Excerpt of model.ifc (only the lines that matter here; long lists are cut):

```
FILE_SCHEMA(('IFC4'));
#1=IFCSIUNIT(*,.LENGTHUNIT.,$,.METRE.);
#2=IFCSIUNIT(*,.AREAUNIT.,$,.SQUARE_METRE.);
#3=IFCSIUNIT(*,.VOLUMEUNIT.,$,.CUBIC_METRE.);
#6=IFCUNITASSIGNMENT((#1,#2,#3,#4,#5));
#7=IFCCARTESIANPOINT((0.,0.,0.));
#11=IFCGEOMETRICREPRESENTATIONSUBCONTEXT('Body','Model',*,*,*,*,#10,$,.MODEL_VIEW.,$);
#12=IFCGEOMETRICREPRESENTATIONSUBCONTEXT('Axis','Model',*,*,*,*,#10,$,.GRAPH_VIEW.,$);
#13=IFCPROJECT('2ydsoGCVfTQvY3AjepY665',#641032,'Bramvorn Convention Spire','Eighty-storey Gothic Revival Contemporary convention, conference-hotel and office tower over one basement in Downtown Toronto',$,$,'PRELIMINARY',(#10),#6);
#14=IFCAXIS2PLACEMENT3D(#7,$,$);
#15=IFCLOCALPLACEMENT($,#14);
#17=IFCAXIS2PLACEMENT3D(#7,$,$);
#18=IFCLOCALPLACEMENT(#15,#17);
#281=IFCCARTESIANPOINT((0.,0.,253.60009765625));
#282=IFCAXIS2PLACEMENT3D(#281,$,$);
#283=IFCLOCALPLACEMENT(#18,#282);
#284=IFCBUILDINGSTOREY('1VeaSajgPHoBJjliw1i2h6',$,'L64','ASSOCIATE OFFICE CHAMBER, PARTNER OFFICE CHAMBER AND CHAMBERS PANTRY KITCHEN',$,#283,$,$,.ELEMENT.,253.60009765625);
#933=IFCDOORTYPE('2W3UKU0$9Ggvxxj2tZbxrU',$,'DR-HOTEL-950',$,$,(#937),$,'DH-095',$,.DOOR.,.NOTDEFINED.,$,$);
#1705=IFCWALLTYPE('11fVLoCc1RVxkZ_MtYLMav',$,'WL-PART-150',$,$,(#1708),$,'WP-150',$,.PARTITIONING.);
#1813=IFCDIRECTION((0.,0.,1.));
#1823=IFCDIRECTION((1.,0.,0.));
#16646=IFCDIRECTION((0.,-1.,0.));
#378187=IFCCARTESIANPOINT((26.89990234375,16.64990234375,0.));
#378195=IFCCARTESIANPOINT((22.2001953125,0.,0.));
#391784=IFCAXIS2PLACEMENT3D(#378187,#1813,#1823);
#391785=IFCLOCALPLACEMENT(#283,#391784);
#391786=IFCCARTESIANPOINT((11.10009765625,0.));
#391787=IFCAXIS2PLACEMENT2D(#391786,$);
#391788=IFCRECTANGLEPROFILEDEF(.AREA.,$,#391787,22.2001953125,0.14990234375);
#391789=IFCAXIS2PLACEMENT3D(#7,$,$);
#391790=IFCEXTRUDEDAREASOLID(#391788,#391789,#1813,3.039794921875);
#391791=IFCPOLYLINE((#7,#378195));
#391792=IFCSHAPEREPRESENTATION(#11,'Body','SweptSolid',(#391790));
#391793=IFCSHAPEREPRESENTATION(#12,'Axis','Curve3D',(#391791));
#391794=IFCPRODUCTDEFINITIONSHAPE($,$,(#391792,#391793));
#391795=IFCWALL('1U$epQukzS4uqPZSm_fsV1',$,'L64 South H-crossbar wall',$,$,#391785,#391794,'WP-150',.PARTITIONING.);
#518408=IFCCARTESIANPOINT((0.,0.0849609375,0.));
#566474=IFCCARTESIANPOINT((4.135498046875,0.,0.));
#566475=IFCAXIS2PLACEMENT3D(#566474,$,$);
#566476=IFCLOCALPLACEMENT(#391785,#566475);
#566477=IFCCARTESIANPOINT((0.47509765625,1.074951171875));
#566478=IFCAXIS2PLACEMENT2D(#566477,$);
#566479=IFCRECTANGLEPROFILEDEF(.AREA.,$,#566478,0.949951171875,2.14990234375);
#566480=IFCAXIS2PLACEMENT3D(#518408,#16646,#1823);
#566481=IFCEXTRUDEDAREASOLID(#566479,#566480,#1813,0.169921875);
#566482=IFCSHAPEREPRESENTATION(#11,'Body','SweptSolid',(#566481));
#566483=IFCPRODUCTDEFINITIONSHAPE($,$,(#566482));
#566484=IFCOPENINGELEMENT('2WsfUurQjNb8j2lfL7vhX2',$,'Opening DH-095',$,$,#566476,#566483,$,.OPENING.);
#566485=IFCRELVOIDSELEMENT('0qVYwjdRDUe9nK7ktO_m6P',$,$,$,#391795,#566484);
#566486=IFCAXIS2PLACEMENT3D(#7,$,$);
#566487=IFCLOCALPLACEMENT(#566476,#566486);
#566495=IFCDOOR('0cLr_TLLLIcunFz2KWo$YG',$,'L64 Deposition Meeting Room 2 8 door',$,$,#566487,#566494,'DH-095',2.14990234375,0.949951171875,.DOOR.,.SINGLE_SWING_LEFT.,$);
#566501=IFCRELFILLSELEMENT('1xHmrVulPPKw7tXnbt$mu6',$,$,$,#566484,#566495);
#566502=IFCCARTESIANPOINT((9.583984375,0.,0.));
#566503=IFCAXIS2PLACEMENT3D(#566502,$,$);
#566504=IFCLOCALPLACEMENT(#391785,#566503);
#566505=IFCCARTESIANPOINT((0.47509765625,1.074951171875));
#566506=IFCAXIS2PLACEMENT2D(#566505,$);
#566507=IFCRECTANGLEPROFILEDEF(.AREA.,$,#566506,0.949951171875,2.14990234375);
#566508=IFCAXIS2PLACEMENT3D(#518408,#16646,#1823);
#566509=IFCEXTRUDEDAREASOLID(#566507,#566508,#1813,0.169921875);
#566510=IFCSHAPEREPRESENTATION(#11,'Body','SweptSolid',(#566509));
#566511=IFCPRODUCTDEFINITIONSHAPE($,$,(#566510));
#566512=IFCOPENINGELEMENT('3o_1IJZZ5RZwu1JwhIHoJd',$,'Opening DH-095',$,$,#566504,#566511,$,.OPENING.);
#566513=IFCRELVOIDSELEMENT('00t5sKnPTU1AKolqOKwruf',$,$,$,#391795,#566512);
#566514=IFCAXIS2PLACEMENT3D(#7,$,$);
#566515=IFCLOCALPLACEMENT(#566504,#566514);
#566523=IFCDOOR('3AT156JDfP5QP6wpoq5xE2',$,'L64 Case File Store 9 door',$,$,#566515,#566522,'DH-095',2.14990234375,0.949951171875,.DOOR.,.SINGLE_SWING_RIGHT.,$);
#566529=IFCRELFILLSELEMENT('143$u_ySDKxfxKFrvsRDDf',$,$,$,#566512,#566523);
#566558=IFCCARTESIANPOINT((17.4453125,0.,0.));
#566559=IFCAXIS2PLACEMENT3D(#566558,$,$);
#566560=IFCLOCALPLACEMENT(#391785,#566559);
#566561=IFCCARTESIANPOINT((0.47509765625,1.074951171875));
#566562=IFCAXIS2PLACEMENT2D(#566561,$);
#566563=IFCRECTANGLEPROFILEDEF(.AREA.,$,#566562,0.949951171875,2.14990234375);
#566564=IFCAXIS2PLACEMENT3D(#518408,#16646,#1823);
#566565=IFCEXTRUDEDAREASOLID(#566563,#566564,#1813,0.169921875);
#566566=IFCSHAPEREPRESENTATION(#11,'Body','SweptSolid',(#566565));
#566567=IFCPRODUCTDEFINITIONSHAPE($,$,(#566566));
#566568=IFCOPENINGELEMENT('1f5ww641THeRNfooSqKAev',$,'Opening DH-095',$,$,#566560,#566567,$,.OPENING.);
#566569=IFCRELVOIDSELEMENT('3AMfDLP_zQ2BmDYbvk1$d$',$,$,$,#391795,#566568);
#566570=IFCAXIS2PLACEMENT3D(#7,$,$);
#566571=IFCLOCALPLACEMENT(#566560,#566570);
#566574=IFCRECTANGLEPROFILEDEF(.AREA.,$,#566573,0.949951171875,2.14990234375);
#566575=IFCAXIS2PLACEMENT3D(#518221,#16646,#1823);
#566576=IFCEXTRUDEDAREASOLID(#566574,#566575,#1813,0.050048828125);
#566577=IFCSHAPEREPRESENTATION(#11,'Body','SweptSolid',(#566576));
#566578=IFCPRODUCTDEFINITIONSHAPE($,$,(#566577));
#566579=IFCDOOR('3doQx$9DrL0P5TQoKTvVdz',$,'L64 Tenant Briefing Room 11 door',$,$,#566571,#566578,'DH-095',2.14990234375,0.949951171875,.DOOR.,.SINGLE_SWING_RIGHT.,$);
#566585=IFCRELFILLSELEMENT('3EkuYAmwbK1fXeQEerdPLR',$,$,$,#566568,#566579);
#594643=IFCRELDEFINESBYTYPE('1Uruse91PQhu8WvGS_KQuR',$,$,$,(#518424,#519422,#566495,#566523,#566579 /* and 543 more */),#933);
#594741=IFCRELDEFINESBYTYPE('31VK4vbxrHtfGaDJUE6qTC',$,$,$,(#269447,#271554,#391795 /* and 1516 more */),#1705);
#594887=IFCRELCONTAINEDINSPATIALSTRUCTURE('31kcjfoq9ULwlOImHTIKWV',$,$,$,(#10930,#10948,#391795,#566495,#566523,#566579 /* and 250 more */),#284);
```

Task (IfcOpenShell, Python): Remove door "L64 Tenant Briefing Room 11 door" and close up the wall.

```python
import ifcopenshell
import ifcopenshell.api.feature
import ifcopenshell.api.root
import ifcopenshell.geom
import ifcopenshell.util.shape

model = ifcopenshell.open("model.ifc")
settings = ifcopenshell.geom.settings()


def volume(element):
    """Net volume in cubic metres, openings subtracted."""
    shape = ifcopenshell.geom.create_shape(settings, element)
    return ifcopenshell.util.shape.get_volume(shape.geometry)


door = model.by_guid("3doQx$9DrL0P5TQoKTvVdz")
opening = door.FillsVoids[0].RelatingOpeningElement
wall = opening.VoidsElements[0].RelatingBuildingElement
before = volume(wall)

ifcopenshell.api.root.remove_product(model, product=door)
ifcopenshell.api.feature.remove_feature(model, feature=opening)

after = volume(wall)

print(f"wall volume {before:.3f} -> {after:.3f} m3")

model.write("model_updated.ifc")
```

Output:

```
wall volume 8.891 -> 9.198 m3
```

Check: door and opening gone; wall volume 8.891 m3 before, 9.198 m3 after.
